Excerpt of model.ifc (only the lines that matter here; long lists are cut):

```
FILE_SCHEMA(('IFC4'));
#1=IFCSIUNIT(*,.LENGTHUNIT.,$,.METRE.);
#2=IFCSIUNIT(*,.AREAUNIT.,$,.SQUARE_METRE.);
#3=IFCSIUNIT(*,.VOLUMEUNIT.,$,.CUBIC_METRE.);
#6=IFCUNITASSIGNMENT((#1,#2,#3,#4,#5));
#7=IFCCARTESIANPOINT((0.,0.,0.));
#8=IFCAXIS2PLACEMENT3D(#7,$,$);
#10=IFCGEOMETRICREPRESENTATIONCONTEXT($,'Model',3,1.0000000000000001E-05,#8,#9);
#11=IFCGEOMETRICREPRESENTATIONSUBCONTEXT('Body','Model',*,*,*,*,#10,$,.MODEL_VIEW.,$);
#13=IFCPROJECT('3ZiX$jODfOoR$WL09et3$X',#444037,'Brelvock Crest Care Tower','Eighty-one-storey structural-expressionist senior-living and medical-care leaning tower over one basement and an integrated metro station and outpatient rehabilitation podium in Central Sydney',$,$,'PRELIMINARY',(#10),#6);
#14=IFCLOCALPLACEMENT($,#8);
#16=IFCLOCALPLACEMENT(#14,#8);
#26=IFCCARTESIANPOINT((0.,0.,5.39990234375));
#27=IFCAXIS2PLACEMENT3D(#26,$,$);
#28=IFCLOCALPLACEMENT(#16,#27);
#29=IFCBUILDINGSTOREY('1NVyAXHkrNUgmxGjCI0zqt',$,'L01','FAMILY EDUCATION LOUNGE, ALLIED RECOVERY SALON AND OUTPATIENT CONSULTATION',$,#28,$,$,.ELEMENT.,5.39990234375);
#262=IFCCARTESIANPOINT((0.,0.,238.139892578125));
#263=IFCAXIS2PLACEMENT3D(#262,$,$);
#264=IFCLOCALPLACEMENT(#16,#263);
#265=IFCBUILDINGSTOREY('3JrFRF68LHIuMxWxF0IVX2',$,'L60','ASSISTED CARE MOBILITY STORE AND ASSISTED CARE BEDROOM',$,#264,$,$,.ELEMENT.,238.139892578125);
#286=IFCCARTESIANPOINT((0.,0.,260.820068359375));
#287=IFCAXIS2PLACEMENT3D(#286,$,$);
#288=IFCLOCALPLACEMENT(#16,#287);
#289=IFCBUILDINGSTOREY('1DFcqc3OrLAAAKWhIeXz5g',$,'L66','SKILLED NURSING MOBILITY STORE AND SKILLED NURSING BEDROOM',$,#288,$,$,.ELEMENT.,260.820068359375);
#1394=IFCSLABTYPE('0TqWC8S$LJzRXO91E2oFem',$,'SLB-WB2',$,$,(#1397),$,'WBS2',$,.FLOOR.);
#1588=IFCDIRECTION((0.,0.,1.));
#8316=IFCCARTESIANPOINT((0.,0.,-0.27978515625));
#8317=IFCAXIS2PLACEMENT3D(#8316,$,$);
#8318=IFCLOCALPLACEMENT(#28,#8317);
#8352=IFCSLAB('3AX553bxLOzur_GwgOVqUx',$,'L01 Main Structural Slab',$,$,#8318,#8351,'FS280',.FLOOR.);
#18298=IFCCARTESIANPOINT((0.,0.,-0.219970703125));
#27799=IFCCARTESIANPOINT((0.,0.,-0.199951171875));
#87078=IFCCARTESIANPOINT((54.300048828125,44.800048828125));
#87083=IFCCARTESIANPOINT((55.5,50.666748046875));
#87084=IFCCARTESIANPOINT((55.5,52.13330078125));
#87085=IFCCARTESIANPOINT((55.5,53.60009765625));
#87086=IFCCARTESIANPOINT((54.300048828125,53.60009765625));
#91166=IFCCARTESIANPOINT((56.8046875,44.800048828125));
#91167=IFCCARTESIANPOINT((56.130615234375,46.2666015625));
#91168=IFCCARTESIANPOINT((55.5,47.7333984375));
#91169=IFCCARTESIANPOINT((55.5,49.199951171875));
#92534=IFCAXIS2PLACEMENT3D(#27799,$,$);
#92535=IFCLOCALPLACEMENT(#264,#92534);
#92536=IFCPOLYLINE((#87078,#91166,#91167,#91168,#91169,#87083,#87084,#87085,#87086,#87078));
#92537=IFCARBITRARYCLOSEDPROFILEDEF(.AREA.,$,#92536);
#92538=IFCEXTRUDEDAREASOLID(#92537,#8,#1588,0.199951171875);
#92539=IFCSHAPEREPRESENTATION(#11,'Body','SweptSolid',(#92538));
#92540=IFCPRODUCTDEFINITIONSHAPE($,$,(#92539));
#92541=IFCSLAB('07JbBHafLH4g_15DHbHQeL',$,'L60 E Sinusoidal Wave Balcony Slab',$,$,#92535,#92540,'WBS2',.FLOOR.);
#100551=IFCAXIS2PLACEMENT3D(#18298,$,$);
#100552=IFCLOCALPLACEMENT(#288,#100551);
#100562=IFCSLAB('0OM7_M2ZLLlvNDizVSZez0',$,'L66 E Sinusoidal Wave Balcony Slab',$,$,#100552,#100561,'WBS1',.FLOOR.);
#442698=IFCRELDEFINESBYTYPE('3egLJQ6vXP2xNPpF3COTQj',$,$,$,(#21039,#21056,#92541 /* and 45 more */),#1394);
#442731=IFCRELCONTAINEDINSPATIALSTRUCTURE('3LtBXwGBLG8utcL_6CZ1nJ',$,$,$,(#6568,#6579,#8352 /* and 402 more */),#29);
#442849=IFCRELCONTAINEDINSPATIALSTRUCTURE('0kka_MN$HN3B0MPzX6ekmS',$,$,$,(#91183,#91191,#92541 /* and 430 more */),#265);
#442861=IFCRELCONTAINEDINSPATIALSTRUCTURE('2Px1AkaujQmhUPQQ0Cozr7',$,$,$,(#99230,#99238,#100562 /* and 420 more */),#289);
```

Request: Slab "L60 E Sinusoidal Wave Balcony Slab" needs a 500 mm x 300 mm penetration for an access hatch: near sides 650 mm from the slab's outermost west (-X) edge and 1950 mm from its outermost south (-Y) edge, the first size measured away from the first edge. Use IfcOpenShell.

```python
import numpy as np
import ifcopenshell
import ifcopenshell.api.feature
import ifcopenshell.api.geometry
import ifcopenshell.api.root
import ifcopenshell.geom
import ifcopenshell.util.placement
import ifcopenshell.util.representation
import ifcopenshell.util.shape
import ifcopenshell.util.unit

model = ifcopenshell.open("model.ifc")
unit_scale = ifcopenshell.util.unit.calculate_unit_scale(model)
settings = ifcopenshell.geom.settings()


def volume(element):
    """Net volume in cubic metres, openings subtracted."""
    shape = ifcopenshell.geom.create_shape(settings, element)
    return ifcopenshell.util.shape.get_volume(shape.geometry)


slab = model.by_id(92541)
before = volume(slab)

# Extent in the slab's own axes, in metres. The edges named are its -X and -Y sides.
slab_shape = ifcopenshell.geom.create_shape(settings, slab)
vertices = ifcopenshell.util.shape.get_vertices(slab_shape.geometry)
x_min, y_min, bottom = vertices.min(axis=0)
top = vertices[:, 2].max()

opening = ifcopenshell.api.root.create_entity(model, ifc_class="IfcOpeningElement", name="Access hatch opening", predefined_type="OPENING")
context = ifcopenshell.util.representation.get_context(model, "Model", "Body", "MODEL_VIEW")
width, depth = 0.5, 0.3
outline = [(0.0, 0.0), (width, 0.0), (width, depth), (0.0, depth), (0.0, 0.0)]
# Overshoot both faces by 50 mm so the cut is clean.
shape = ifcopenshell.api.geometry.add_slab_representation(
    model, context=context, depth=top - bottom + 0.1, polyline=outline
)
ifcopenshell.api.geometry.assign_representation(model, product=opening, representation=shape)

matrix = ifcopenshell.util.placement.get_local_placement(slab.ObjectPlacement)
matrix[:, 3] = matrix @ np.append(np.array([x_min + 0.65, y_min + 1.95, bottom - 0.05]) / unit_scale, 1.0)
ifcopenshell.api.geometry.edit_object_placement(model, product=opening, matrix=matrix, is_si=False)
ifcopenshell.api.feature.add_feature(model, feature=opening, element=slab)

after = volume(slab)

print(f"slab volume {before:.3f} -> {after:.3f} m3")

model.write("model_edited.ifc")
```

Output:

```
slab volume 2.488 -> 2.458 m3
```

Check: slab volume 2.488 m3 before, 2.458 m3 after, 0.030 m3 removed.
